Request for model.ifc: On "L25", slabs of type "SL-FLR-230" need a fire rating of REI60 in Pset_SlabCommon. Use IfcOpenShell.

First a look at what the model holds.

```python
import ifcopenshell
import ifcopenshell.util.element

model = ifcopenshell.open("model.ifc")
print(model.schema)
storey = next(s for s in model.by_type("IfcBuildingStorey") if s.Name == "L25")
slabs = [e for e in ifcopenshell.util.element.get_decomposition(storey) if e.is_a("IfcSlab")]
seen = {}
for e in slabs:
    element_type = ifcopenshell.util.element.get_type(e)
    key = (element_type.Name if element_type != e and element_type else None, ifcopenshell.util.element.get_pset(e, "Pset_SlabCommon", "FireRating"))
    seen[key] = seen.get(key, 0) + 1
for (name, value), count in sorted(seen.items(), key=str):
    print(count, "x", name, "|", value)
```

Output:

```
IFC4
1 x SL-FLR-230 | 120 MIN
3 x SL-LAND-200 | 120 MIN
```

```python
import ifcopenshell
import ifcopenshell.api.pset
import ifcopenshell.util.element

model = ifcopenshell.open("model.ifc")

storey = next(s for s in model.by_type("IfcBuildingStorey") if s.Name == "L25")
slabs = [e for e in ifcopenshell.util.element.get_decomposition(storey) if e.is_a("IfcSlab")]

count = 0
for e in slabs:
    element_type = ifcopenshell.util.element.get_type(e)
    if element_type in (None, e) or element_type.Name != "SL-FLR-230":
        continue
    found = ifcopenshell.util.element.get_pset(e, "Pset_SlabCommon", should_inherit=False)
    if found:
        pset = model.by_id(found["id"])
        if len(ifcopenshell.util.element.get_elements_by_pset(pset)) > 1:
            pset = ifcopenshell.api.pset.unshare_pset(model, products=[e], pset=pset)[0]
    else:
        pset = ifcopenshell.api.pset.add_pset(model, product=e, name="Pset_SlabCommon")
    ifcopenshell.api.pset.edit_pset(model, pset=pset, properties={"FireRating": "REI60"})
    count += 1

print(count, "slabs updated")

model.write("model_edited.ifc")
```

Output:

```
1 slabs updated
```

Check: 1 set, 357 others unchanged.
